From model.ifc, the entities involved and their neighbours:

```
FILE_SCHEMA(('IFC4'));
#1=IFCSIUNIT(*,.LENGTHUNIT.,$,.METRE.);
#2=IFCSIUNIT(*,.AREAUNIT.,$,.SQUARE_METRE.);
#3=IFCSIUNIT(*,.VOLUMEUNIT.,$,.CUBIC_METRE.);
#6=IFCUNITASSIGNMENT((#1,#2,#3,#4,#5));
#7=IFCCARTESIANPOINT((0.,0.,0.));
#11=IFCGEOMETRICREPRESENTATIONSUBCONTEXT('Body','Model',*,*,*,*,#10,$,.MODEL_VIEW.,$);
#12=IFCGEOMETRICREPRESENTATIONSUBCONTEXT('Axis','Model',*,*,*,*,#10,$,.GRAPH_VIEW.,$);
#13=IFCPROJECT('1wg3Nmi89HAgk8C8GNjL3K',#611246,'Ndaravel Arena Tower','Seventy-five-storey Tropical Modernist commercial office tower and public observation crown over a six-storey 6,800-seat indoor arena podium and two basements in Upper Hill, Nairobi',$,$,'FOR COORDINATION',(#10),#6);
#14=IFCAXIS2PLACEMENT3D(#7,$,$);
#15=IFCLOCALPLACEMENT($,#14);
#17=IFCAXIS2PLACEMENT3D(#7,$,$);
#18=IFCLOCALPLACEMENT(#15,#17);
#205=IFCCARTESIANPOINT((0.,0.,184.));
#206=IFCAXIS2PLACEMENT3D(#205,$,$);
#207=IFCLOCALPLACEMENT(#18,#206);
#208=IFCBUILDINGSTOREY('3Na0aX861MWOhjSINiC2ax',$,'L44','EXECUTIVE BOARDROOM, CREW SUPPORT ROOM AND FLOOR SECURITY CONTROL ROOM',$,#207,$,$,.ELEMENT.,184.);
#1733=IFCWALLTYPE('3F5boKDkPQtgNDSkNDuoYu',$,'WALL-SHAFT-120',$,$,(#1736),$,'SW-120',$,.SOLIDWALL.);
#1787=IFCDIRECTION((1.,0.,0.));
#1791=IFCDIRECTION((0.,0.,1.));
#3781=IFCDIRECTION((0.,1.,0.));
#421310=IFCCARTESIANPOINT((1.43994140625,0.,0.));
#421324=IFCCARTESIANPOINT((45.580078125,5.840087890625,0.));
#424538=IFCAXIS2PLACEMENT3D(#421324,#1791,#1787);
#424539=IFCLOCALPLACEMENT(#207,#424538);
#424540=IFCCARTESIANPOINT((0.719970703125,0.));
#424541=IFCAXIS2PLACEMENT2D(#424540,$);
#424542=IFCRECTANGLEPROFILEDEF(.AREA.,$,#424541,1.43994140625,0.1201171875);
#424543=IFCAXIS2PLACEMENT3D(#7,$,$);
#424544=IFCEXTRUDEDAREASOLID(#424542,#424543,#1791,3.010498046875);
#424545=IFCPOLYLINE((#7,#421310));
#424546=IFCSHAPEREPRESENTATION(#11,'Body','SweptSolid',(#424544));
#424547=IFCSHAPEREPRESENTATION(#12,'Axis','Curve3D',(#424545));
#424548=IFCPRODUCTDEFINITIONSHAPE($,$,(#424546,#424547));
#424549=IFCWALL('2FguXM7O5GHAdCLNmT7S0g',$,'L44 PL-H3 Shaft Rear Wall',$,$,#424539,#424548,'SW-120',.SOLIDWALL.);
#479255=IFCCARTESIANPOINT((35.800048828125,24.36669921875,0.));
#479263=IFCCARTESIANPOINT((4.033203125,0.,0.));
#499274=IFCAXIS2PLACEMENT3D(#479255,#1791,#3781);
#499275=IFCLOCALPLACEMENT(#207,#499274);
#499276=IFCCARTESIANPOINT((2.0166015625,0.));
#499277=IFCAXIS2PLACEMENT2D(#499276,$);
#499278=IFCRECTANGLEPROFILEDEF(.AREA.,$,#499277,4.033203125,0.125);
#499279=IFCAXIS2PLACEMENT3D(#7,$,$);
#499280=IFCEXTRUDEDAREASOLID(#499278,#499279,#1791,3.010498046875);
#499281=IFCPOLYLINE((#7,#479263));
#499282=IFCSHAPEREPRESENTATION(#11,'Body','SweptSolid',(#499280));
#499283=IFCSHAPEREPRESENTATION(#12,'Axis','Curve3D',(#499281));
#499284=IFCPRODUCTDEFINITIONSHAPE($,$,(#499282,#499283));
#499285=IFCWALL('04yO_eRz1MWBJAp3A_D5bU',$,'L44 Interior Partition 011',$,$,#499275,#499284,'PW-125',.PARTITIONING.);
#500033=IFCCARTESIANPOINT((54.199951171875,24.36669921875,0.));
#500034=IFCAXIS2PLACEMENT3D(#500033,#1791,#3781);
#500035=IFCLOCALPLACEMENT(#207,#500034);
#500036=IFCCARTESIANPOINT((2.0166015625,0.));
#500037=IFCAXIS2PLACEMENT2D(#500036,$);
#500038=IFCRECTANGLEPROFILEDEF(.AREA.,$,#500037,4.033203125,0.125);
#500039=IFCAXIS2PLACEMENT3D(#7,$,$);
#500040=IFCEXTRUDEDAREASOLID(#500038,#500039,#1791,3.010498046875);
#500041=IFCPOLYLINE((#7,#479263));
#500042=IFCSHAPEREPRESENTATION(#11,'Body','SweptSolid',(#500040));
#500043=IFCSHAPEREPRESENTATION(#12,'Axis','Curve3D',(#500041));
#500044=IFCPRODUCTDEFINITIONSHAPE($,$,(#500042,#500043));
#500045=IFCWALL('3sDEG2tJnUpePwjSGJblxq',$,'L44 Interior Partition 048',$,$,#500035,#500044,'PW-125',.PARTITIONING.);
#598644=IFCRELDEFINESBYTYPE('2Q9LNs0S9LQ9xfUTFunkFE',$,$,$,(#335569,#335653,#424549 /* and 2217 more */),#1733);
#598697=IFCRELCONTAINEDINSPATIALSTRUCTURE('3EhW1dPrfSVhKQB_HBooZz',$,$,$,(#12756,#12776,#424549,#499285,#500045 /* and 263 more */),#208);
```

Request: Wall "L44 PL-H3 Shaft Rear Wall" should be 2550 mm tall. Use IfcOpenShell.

```python
import ifcopenshell
import ifcopenshell.geom
import ifcopenshell.util.representation
import ifcopenshell.util.shape

model = ifcopenshell.open("model.ifc")
settings = ifcopenshell.geom.settings()


def volume(element):
    """Net volume in cubic metres, openings subtracted."""
    shape = ifcopenshell.geom.create_shape(settings, element)
    return ifcopenshell.util.shape.get_volume(shape.geometry)


wall = model.by_guid("2FguXM7O5GHAdCLNmT7S0g")
before = volume(wall)

body = ifcopenshell.util.representation.get_representation(wall, "Model", "Body")
solid = body.Items[0]
old_height = solid.Depth
solid.Depth = 2.55
after = volume(wall)

print(f"height {old_height:g} -> {solid.Depth:g}, volume {before:.3f} -> {after:.3f} m3")

model.write("model_edited.ifc")
```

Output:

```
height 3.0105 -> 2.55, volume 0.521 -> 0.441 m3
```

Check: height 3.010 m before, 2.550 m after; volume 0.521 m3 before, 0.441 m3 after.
